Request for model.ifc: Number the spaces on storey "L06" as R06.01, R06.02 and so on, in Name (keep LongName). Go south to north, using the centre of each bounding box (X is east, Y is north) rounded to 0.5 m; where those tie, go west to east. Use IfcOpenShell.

First a look at what the model holds.

```python
import ifcopenshell
import ifcopenshell.util.element
import ifcopenshell.util.placement

model = ifcopenshell.open("model.ifc")
print(model.schema)
storey = next(s for s in model.by_type("IfcBuildingStorey") if s.Name == "L06")
spaces = [e for e in ifcopenshell.util.element.get_decomposition(storey) if e.is_a("IfcSpace")]
for e in sorted(spaces, key=lambda e: e.id()):
    origin = ifcopenshell.util.placement.get_local_placement(e.ObjectPlacement)[:3, 3]
    print(e.id(), e.Name, e.LongName, origin.round(2) + 0.0, sep=" | ")
```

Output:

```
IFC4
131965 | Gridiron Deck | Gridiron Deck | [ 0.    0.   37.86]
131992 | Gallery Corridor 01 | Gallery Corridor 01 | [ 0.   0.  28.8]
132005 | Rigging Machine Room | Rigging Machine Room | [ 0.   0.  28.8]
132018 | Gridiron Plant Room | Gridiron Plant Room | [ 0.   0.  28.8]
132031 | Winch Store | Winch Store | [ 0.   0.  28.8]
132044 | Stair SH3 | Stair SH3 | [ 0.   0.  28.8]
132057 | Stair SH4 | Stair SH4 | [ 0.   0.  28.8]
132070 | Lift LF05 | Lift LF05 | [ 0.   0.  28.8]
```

```python
import ifcopenshell
import ifcopenshell.geom
import ifcopenshell.util.element
import ifcopenshell.util.shape

model = ifcopenshell.open("model.ifc")
settings = ifcopenshell.geom.settings()
settings.set("use-world-coords", True)


def centre(element):
    shape = ifcopenshell.geom.create_shape(settings, element)
    return ifcopenshell.util.shape.get_bbox_centroid(shape.geometry)


storey = next(s for s in model.by_type("IfcBuildingStorey") if s.Name == "L06")
spaces = [e for e in ifcopenshell.util.element.get_decomposition(storey) if e.is_a("IfcSpace")]

# Insertion points can sit at a corner or the storey origin, so sort by the geometry (in metres).
centres = {e: centre(e) for e in spaces}
spaces.sort(key=lambda e: (round(centres[e][1] / 0.5), centres[e][0]))

for i, e in enumerate(spaces, start=1):
    number = f"R06.{i:02d}"
    e.Name = number
    print(e.id(), number)

model.write("model_rev.ifc")
```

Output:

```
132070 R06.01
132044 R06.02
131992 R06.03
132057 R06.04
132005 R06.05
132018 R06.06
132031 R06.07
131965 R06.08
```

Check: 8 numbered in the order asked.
